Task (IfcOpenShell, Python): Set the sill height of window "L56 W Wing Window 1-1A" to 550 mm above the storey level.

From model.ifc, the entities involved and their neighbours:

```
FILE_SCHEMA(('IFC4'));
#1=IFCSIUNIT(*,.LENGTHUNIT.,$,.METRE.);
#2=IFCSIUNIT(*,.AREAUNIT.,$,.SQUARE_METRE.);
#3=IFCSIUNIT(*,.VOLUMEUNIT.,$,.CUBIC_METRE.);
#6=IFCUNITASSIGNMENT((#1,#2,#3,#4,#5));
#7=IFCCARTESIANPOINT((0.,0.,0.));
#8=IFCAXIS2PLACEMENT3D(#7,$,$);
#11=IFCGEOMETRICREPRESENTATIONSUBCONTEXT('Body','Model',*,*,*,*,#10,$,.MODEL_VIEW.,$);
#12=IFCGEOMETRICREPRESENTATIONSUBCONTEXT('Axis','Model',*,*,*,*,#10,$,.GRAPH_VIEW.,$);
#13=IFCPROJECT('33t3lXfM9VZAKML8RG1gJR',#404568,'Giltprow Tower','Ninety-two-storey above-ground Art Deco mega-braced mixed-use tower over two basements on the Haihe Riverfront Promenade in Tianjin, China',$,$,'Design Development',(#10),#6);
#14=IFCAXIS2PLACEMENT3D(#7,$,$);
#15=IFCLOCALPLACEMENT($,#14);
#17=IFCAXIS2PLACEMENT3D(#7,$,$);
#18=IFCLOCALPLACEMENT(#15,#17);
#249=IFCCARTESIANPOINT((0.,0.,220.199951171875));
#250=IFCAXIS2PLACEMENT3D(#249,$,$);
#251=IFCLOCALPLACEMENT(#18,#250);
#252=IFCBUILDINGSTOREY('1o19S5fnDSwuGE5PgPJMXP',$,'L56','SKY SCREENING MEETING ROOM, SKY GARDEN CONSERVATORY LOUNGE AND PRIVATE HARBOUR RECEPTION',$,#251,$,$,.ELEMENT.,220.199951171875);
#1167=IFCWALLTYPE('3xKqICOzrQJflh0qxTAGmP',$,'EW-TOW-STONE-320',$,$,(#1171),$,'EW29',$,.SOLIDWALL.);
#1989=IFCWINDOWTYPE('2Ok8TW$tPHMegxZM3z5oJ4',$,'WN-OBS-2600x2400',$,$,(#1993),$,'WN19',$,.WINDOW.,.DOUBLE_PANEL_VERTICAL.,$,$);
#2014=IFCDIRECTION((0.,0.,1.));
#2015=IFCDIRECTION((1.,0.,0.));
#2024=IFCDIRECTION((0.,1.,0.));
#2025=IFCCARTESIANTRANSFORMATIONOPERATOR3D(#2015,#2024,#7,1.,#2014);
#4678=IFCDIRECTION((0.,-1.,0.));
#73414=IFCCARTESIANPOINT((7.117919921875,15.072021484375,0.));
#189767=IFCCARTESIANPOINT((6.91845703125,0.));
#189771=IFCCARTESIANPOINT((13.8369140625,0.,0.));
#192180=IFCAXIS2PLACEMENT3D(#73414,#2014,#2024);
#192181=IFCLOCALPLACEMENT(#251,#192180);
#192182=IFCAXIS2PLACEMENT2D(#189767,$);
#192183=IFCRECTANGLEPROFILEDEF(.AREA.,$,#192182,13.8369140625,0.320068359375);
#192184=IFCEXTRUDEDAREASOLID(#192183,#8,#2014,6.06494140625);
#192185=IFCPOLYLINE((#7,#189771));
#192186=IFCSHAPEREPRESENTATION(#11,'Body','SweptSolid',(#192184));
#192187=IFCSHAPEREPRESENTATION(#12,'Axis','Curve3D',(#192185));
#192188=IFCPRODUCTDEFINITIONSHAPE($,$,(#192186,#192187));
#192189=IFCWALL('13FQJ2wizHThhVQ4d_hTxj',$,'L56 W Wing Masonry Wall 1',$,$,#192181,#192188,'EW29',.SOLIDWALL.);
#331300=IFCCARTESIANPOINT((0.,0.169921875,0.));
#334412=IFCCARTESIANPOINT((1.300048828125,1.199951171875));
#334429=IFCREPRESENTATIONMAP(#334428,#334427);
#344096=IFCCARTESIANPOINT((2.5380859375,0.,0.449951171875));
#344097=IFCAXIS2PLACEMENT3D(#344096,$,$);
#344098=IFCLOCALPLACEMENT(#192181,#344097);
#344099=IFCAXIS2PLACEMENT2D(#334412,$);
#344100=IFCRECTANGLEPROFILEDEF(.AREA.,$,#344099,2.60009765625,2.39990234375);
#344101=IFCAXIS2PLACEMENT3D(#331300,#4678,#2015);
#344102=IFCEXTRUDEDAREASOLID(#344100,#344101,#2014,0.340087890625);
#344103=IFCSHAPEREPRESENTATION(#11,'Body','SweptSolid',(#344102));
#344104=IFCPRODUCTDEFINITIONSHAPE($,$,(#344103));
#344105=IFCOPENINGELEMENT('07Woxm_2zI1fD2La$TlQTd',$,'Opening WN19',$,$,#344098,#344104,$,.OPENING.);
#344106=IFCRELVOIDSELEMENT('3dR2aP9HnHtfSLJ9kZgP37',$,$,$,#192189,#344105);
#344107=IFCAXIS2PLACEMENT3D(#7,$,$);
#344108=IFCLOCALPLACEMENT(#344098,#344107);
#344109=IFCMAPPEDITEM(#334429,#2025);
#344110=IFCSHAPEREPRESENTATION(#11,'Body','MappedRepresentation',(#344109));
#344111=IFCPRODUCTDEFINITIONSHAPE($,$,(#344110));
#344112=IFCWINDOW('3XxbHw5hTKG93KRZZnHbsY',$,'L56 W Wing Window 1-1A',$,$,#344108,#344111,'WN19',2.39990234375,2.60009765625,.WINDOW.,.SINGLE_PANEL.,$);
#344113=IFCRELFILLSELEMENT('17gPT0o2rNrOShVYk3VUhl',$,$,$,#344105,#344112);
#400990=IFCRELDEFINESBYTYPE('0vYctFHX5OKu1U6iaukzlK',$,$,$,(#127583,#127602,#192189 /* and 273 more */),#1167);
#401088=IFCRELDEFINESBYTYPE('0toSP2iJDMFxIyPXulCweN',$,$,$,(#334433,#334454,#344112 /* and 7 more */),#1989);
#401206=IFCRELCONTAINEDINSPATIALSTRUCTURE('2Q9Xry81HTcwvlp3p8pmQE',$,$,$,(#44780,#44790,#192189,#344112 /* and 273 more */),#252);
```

```python
import numpy as np
import ifcopenshell
import ifcopenshell.api.geometry
import ifcopenshell.geom
import ifcopenshell.util.element
import ifcopenshell.util.placement
import ifcopenshell.util.shape
import ifcopenshell.util.unit

model = ifcopenshell.open("model.ifc")
unit_scale = ifcopenshell.util.unit.calculate_unit_scale(model)

window = model.by_id(344112)
opening = window.FillsVoids[0].RelatingOpeningElement
storey = ifcopenshell.util.element.get_container(window, ifc_class="IfcBuildingStorey")
level = ifcopenshell.util.placement.get_local_placement(storey.ObjectPlacement)[2, 3]

# The opening's origin need not be at the sill, so measure its lowest point.
shape = ifcopenshell.geom.create_shape(ifcopenshell.geom.settings(), opening)
bottom = ifcopenshell.util.shape.get_shape_bottom_elevation(shape, shape.geometry) / unit_scale
dz = level + 0.55 / unit_scale - bottom

shift = np.array([0.0, 0.0, dz])
# The window is placed relative to its opening, so it follows when the opening moves.
matrix = ifcopenshell.util.placement.get_local_placement(opening.ObjectPlacement)
matrix[:3, 3] += shift
ifcopenshell.api.geometry.edit_object_placement(
    model, product=opening, matrix=matrix, is_si=False, should_transform_children=True
)

print(f"moved by {dz * unit_scale:+.3f} m")

model.write("model-out.ifc")
```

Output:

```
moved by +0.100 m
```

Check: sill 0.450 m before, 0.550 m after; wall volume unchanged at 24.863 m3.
